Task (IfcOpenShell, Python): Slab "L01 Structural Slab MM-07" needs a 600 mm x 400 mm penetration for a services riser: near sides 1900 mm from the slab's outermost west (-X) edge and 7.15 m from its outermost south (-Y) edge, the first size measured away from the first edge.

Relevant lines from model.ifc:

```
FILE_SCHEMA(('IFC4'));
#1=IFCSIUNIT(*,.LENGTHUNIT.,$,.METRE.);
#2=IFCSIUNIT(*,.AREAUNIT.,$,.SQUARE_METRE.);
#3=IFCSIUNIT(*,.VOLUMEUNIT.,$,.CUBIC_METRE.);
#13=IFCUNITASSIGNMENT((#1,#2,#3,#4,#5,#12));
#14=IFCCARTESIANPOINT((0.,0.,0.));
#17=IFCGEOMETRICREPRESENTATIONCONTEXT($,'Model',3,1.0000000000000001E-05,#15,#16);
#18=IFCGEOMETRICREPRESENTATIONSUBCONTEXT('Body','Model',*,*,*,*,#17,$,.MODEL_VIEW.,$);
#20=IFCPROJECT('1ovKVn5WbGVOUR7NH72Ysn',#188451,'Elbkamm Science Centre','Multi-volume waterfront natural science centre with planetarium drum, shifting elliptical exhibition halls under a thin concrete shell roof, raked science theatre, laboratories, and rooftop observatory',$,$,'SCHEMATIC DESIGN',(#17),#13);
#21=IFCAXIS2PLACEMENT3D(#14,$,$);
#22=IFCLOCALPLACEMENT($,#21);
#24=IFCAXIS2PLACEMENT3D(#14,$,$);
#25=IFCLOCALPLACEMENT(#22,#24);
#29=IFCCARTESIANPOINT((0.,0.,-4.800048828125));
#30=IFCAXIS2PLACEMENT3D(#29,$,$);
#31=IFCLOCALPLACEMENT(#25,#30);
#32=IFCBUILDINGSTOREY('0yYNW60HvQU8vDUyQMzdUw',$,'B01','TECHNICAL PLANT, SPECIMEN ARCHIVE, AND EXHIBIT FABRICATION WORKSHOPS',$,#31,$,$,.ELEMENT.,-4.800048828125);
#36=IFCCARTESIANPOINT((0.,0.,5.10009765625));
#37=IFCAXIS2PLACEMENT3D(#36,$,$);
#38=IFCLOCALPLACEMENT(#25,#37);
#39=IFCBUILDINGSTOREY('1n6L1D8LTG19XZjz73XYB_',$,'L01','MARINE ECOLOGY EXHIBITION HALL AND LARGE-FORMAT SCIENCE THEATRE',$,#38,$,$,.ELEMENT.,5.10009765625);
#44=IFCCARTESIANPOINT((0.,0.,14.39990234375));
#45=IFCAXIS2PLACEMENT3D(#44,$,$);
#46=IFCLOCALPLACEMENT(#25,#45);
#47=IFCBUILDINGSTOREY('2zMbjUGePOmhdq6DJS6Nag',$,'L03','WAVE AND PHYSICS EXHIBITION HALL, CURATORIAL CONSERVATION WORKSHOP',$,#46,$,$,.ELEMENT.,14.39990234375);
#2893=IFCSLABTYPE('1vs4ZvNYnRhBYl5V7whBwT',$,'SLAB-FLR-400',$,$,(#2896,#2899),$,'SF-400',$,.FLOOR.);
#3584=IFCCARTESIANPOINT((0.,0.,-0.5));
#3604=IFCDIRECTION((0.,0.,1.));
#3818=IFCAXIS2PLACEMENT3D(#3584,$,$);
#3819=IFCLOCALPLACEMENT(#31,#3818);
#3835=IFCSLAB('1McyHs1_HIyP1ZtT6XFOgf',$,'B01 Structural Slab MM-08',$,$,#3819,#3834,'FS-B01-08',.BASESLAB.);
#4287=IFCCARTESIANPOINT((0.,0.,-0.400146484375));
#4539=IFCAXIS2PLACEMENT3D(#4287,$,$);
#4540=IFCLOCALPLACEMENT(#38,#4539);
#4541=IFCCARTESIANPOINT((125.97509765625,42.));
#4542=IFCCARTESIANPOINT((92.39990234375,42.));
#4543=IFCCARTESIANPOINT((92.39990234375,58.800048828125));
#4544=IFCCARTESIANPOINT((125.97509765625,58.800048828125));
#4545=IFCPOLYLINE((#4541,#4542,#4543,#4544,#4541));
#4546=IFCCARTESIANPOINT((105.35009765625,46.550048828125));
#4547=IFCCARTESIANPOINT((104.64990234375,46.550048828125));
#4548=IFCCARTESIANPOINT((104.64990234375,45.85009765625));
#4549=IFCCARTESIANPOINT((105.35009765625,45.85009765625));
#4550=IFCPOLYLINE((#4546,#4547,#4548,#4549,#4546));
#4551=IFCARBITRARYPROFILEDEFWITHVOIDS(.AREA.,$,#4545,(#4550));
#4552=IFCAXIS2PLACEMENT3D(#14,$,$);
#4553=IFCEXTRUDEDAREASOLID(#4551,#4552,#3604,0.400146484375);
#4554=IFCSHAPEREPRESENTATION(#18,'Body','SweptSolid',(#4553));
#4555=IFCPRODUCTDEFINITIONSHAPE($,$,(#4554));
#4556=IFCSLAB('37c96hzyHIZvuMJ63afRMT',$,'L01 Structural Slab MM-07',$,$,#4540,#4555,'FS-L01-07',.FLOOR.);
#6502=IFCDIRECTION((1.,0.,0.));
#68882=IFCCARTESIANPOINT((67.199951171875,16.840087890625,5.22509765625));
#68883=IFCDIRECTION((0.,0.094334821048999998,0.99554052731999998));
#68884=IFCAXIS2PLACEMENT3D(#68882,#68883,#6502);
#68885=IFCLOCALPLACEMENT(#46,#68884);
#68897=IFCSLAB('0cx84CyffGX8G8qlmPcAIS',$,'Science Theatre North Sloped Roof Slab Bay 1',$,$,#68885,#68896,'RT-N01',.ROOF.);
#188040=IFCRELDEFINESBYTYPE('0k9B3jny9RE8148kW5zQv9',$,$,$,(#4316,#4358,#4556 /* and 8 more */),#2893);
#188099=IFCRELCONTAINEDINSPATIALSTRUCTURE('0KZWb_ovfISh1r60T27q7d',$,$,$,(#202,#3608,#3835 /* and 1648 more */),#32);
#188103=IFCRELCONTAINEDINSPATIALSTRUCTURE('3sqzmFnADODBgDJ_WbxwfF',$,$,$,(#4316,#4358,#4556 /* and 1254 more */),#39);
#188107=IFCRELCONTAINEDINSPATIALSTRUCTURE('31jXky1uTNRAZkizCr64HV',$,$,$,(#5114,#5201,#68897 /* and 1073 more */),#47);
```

```python
import numpy as np
import ifcopenshell
import ifcopenshell.api.feature
import ifcopenshell.api.geometry
import ifcopenshell.api.root
import ifcopenshell.geom
import ifcopenshell.util.placement
import ifcopenshell.util.representation
import ifcopenshell.util.shape
import ifcopenshell.util.unit

model = ifcopenshell.open("model.ifc")
unit_scale = ifcopenshell.util.unit.calculate_unit_scale(model)
settings = ifcopenshell.geom.settings()


def volume(element):
    """Net volume in cubic metres, openings subtracted."""
    shape = ifcopenshell.geom.create_shape(settings, element)
    return ifcopenshell.util.shape.get_volume(shape.geometry)


slab = model.by_id(4556)
before = volume(slab)

# Extent in the slab's own axes, in metres. The edges named are its -X and -Y sides.
slab_shape = ifcopenshell.geom.create_shape(settings, slab)
vertices = ifcopenshell.util.shape.get_vertices(slab_shape.geometry)
x_min, y_min, bottom = vertices.min(axis=0)
top = vertices[:, 2].max()

opening = ifcopenshell.api.root.create_entity(model, ifc_class="IfcOpeningElement", name="Services riser opening", predefined_type="OPENING")
context = ifcopenshell.util.representation.get_context(model, "Model", "Body", "MODEL_VIEW")
width, depth = 0.6, 0.4
outline = [(0.0, 0.0), (width, 0.0), (width, depth), (0.0, depth), (0.0, 0.0)]
# Overshoot both faces by 50 mm so the cut is clean.
shape = ifcopenshell.api.geometry.add_slab_representation(
    model, context=context, depth=top - bottom + 0.1, polyline=outline
)
ifcopenshell.api.geometry.assign_representation(model, product=opening, representation=shape)

matrix = ifcopenshell.util.placement.get_local_placement(slab.ObjectPlacement)
matrix[:, 3] = matrix @ np.append(np.array([x_min + 1.9, y_min + 7.15, bottom - 0.05]) / unit_scale, 1.0)
ifcopenshell.api.geometry.edit_object_placement(model, product=opening, matrix=matrix, is_si=False)
ifcopenshell.api.feature.add_feature(model, feature=opening, element=slab)

after = volume(slab)

print(f"slab volume {before:.3f} -> {after:.3f} m3")

model.write("model_edited.ifc")
```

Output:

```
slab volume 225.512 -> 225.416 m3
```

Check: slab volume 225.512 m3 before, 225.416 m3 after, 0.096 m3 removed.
